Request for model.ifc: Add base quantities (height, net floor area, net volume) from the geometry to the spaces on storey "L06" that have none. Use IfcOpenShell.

First a look at what the model holds.

```python
import ifcopenshell
import ifcopenshell.util.element
import ifcopenshell.util.unit

model = ifcopenshell.open("model.ifc")
print(model.schema)
for unit_type in ("LENGTHUNIT", "AREAUNIT", "VOLUMEUNIT"):
    print(unit_type, ifcopenshell.util.unit.calculate_unit_scale(model, unit_type))
storey = next(s for s in model.by_type("IfcBuildingStorey") if s.Name == "L06")
spaces = [e for e in ifcopenshell.util.element.get_decomposition(storey) if e.is_a("IfcSpace")]
for e in sorted(spaces, key=lambda e: e.id()):
    print(e.id(), e.is_a(), e.Name, list(ifcopenshell.util.element.get_psets(e, qtos_only=True)), sep=" | ")
```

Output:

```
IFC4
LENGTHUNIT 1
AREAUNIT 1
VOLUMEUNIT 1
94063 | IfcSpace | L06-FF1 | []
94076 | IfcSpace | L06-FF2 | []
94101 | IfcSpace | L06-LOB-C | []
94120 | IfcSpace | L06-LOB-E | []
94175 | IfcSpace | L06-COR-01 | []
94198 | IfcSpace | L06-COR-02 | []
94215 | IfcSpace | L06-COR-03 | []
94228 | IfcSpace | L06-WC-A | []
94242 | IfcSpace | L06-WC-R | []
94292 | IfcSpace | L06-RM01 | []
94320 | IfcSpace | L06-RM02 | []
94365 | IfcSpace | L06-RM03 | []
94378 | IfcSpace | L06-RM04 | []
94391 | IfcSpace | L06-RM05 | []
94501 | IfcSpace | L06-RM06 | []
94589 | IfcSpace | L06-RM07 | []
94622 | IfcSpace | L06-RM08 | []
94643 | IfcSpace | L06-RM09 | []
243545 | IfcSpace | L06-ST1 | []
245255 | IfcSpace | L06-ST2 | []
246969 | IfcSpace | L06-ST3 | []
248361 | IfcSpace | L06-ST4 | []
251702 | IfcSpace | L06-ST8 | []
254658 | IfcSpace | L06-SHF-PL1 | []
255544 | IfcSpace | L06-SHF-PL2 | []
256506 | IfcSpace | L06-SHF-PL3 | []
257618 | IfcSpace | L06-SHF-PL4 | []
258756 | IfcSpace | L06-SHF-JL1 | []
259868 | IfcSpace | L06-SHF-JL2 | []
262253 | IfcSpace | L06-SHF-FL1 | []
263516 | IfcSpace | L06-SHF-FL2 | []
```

```python
import ifcopenshell
import ifcopenshell.api.pset
import ifcopenshell.geom
import ifcopenshell.util.element
import ifcopenshell.util.shape
import ifcopenshell.util.unit

model = ifcopenshell.open("model.ifc")
unit_scale = ifcopenshell.util.unit.calculate_unit_scale(model)
area_scale = ifcopenshell.util.unit.calculate_unit_scale(model, "AREAUNIT")
volume_scale = ifcopenshell.util.unit.calculate_unit_scale(model, "VOLUMEUNIT")
settings = ifcopenshell.geom.settings()

storey = next(s for s in model.by_type("IfcBuildingStorey") if s.Name == "L06")
spaces = [e for e in ifcopenshell.util.element.get_decomposition(storey) if e.is_a("IfcSpace")]

for e in sorted(spaces, key=lambda e: e.id()):
    if ifcopenshell.util.element.get_psets(e, qtos_only=True, should_inherit=False):
        continue
    # Geometry comes back in metres, in the element's own axes.
    shape = ifcopenshell.geom.create_shape(settings, e)
    values = {
        "Height": ifcopenshell.util.shape.get_z(shape.geometry) / unit_scale,
        "NetFloorArea": ifcopenshell.util.shape.get_footprint_area(shape.geometry) / area_scale,
        "NetVolume": ifcopenshell.util.shape.get_volume(shape.geometry) / volume_scale,
    }
    qto = ifcopenshell.api.pset.add_qto(model, product=e, name="Qto_SpaceBaseQuantities")
    ifcopenshell.api.pset.edit_qto(model, qto=qto, properties=values)
    print(e.id(), {k: round(v, 3) for k, v in values.items()})

model.write("model_v2.ifc")
```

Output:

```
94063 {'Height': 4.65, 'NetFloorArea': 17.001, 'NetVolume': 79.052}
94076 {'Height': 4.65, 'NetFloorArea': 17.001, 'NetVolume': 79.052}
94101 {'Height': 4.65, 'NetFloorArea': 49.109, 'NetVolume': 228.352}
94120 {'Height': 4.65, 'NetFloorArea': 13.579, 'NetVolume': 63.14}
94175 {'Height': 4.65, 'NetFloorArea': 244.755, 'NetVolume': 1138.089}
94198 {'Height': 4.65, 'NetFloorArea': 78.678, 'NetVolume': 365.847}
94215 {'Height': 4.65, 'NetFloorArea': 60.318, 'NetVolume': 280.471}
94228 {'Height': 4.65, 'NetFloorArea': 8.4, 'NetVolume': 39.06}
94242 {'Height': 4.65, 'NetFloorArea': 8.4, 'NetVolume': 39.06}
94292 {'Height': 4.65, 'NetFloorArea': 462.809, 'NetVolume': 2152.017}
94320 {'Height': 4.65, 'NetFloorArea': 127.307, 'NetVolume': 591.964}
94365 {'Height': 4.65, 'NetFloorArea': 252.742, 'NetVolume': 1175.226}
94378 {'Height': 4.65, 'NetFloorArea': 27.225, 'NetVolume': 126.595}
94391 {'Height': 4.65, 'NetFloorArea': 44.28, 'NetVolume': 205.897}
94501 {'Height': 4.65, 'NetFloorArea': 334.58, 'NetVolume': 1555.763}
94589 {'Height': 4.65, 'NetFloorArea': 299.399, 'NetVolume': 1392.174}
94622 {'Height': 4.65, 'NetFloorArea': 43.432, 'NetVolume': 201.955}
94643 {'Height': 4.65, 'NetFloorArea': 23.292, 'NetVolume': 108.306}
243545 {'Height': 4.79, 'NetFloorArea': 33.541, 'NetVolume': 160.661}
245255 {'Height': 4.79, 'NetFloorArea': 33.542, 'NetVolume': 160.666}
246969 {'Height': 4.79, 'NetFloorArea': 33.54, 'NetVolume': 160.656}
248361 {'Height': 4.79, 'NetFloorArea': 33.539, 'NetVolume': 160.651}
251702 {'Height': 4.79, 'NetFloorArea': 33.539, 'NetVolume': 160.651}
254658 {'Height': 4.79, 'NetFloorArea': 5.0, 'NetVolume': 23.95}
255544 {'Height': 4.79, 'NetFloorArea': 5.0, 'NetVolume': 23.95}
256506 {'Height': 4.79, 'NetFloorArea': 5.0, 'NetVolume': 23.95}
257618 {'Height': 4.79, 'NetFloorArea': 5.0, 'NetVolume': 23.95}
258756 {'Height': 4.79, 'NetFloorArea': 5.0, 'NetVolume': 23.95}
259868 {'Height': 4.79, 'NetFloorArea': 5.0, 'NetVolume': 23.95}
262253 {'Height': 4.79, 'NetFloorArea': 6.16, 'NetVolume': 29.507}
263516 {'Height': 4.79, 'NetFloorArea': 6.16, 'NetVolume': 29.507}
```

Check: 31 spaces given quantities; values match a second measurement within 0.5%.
